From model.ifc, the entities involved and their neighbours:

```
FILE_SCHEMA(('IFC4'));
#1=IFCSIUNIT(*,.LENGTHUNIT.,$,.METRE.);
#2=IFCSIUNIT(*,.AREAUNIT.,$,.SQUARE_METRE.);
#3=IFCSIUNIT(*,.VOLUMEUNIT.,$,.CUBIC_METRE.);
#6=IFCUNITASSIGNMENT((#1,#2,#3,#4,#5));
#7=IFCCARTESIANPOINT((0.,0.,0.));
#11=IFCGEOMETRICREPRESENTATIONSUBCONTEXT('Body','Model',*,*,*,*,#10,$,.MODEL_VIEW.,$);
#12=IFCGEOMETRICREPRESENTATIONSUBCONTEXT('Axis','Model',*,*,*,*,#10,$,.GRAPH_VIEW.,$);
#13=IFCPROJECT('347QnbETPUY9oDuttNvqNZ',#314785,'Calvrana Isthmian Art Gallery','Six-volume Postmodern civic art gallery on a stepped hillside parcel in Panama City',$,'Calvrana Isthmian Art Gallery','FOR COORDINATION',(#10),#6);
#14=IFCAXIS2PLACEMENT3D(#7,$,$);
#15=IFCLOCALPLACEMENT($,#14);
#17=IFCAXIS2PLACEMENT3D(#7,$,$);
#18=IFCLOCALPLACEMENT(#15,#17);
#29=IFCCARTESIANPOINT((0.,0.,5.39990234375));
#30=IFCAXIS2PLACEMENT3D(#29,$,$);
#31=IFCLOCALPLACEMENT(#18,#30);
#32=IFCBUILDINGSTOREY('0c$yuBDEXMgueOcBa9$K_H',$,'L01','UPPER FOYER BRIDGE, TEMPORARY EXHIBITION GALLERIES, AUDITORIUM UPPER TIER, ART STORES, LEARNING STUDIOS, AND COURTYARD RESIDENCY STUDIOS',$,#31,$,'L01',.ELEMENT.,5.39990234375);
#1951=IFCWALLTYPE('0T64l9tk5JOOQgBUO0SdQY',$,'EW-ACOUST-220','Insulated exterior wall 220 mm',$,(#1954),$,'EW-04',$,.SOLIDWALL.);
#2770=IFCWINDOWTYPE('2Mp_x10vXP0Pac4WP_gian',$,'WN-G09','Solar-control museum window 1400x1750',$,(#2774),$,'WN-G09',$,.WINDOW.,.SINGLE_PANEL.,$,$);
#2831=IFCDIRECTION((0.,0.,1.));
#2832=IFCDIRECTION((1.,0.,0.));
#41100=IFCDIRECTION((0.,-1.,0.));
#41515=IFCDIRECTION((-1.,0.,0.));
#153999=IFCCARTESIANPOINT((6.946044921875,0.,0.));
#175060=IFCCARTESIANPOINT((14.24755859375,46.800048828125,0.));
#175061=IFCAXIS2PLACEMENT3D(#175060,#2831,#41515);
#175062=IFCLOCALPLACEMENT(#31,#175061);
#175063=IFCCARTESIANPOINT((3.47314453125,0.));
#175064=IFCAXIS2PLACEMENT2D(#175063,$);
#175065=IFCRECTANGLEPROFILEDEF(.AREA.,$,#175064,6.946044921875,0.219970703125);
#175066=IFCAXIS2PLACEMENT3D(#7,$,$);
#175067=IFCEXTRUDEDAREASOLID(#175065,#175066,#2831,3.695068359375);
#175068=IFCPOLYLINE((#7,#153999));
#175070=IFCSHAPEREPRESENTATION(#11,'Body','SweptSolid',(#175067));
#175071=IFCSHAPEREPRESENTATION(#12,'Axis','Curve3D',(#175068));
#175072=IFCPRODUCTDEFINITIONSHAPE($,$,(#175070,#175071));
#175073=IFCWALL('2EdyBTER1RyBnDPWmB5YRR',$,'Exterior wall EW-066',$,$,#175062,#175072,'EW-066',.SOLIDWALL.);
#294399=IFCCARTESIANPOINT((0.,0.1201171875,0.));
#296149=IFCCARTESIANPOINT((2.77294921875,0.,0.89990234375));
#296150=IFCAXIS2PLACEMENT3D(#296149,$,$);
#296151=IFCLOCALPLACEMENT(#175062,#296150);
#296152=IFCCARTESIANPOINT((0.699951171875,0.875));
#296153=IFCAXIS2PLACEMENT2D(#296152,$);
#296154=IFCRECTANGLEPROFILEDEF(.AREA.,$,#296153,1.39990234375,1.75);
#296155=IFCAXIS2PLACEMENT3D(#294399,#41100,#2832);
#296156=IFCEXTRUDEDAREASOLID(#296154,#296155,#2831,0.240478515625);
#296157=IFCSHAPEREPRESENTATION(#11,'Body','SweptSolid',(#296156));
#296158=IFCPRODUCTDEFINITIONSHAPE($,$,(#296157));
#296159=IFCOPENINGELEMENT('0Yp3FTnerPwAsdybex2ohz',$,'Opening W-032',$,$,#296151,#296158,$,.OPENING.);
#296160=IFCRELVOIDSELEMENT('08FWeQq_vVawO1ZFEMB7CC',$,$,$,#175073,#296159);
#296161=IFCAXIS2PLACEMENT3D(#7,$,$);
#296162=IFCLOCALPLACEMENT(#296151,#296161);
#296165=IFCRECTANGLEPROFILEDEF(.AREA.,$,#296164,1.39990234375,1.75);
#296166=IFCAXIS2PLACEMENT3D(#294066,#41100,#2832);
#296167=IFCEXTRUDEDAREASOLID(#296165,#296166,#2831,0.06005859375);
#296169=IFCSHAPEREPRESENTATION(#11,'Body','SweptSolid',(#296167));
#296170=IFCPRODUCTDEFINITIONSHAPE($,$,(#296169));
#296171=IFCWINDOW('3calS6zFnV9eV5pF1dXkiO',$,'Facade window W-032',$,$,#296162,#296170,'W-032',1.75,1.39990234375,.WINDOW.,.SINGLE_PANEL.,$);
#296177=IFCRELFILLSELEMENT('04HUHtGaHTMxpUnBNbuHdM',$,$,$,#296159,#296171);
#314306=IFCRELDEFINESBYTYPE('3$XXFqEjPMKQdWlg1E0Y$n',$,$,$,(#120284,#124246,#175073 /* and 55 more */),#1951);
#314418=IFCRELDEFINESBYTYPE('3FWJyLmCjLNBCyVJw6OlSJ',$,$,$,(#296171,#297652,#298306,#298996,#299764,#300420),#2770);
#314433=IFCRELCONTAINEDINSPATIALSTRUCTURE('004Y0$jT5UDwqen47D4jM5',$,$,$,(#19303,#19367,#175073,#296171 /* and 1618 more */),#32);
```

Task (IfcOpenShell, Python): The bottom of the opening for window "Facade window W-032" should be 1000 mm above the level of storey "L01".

```python
import numpy as np
import ifcopenshell
import ifcopenshell.api.geometry
import ifcopenshell.geom
import ifcopenshell.util.element
import ifcopenshell.util.placement
import ifcopenshell.util.shape
import ifcopenshell.util.unit

model = ifcopenshell.open("model.ifc")
unit_scale = ifcopenshell.util.unit.calculate_unit_scale(model)

window = model.by_guid("3calS6zFnV9eV5pF1dXkiO")
opening = window.FillsVoids[0].RelatingOpeningElement
storey = ifcopenshell.util.element.get_container(window, ifc_class="IfcBuildingStorey")
level = ifcopenshell.util.placement.get_local_placement(storey.ObjectPlacement)[2, 3]

# The opening's origin need not be at the sill, so measure its lowest point.
shape = ifcopenshell.geom.create_shape(ifcopenshell.geom.settings(), opening)
bottom = ifcopenshell.util.shape.get_shape_bottom_elevation(shape, shape.geometry) / unit_scale
dz = level + 1 / unit_scale - bottom

shift = np.array([0.0, 0.0, dz])
# The window is placed relative to its opening, so it follows when the opening moves.
matrix = ifcopenshell.util.placement.get_local_placement(opening.ObjectPlacement)
matrix[:3, 3] += shift
ifcopenshell.api.geometry.edit_object_placement(
    model, product=opening, matrix=matrix, is_si=False, should_transform_children=True
)

print(f"moved by {dz * unit_scale:+.3f} m")

model.write("model_updated.ifc")
```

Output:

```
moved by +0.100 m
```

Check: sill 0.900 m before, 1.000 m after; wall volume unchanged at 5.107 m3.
